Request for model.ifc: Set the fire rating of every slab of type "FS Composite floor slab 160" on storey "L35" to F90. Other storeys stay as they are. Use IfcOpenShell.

First a look at what the model holds.

```python
import ifcopenshell
import ifcopenshell.util.element

model = ifcopenshell.open("model.ifc")
print(model.schema)
storey = next(s for s in model.by_type("IfcBuildingStorey") if s.Name == "L35")
slabs = [e for e in ifcopenshell.util.element.get_decomposition(storey) if e.is_a("IfcSlab")]
seen = {}
for e in slabs:
    element_type = ifcopenshell.util.element.get_type(e)
    key = (element_type.Name if element_type != e and element_type else None, ifcopenshell.util.element.get_pset(e, "Pset_SlabCommon", "FireRating"))
    seen[key] = seen.get(key, 0) + 1
for (name, value), count in sorted(seen.items(), key=str):
    print(count, "x", name, "|", value)
```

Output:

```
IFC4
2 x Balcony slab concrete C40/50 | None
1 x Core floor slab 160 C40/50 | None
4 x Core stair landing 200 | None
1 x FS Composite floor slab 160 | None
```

```python
import ifcopenshell
import ifcopenshell.api.pset
import ifcopenshell.util.element

model = ifcopenshell.open("model.ifc")

storey = next(s for s in model.by_type("IfcBuildingStorey") if s.Name == "L35")
slabs = [e for e in ifcopenshell.util.element.get_decomposition(storey) if e.is_a("IfcSlab")]

count = 0
for e in slabs:
    element_type = ifcopenshell.util.element.get_type(e)
    if element_type in (None, e) or element_type.Name != "FS Composite floor slab 160":
        continue
    found = ifcopenshell.util.element.get_pset(e, "Pset_SlabCommon", should_inherit=False)
    if found:
        pset = model.by_id(found["id"])
        if len(ifcopenshell.util.element.get_elements_by_pset(pset)) > 1:
            pset = ifcopenshell.api.pset.unshare_pset(model, products=[e], pset=pset)[0]
    else:
        pset = ifcopenshell.api.pset.add_pset(model, product=e, name="Pset_SlabCommon")
    ifcopenshell.api.pset.edit_pset(model, pset=pset, properties={"FireRating": "F90"})
    count += 1

print(count, "slabs updated")

model.write("model-out.ifc")
```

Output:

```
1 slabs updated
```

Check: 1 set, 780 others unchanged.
